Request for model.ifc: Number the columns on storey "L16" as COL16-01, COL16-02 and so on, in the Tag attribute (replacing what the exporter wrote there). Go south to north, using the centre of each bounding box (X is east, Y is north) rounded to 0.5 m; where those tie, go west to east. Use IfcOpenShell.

First a look at what the model holds.

```python
import ifcopenshell
import ifcopenshell.util.element
import ifcopenshell.util.placement

model = ifcopenshell.open("model.ifc")
print(model.schema)
storey = next(s for s in model.by_type("IfcBuildingStorey") if s.Name == "L16")
columns = [e for e in ifcopenshell.util.element.get_decomposition(storey) if e.is_a("IfcColumn")]
for e in sorted(columns, key=lambda e: e.id()):
    origin = ifcopenshell.util.placement.get_local_placement(e.ObjectPlacement)[:3, 3]
    print(e.id(), e.Tag, e.Name, origin.round(2) + 0.0, sep=" | ")
```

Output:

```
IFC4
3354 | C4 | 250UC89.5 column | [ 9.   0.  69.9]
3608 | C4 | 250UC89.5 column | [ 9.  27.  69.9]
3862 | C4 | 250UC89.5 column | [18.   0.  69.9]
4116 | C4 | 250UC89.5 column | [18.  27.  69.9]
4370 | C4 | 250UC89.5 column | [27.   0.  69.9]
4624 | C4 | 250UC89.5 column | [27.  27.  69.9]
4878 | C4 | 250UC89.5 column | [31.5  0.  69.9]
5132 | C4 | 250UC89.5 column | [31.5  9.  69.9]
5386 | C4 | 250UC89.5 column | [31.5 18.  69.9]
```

```python
import ifcopenshell
import ifcopenshell.geom
import ifcopenshell.util.element
import ifcopenshell.util.shape

model = ifcopenshell.open("model.ifc")
settings = ifcopenshell.geom.settings()
settings.set("use-world-coords", True)


def centre(element):
    shape = ifcopenshell.geom.create_shape(settings, element)
    return ifcopenshell.util.shape.get_bbox_centroid(shape.geometry)


storey = next(s for s in model.by_type("IfcBuildingStorey") if s.Name == "L16")
columns = [e for e in ifcopenshell.util.element.get_decomposition(storey) if e.is_a("IfcColumn")]

# Insertion points can sit at a corner or the storey origin, so sort by the geometry (in metres).
centres = {e: centre(e) for e in columns}
columns.sort(key=lambda e: (round(centres[e][1] / 0.5), centres[e][0]))

for i, e in enumerate(columns, start=1):
    number = f"COL16-{i:02d}"
    e.Tag = number
    print(e.id(), number)

model.write("model-out.ifc")
```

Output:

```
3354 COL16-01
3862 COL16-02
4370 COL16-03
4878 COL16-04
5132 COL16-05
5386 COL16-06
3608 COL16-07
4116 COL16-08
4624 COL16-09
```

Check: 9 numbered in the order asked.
